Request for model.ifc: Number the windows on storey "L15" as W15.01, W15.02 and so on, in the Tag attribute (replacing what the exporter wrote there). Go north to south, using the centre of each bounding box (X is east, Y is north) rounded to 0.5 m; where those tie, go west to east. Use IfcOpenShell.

First a look at what the model holds.

```python
import ifcopenshell
import ifcopenshell.util.element
import ifcopenshell.util.placement

model = ifcopenshell.open("model.ifc")
print(model.schema)
storey = next(s for s in model.by_type("IfcBuildingStorey") if s.Name == "L15")
windows = [e for e in ifcopenshell.util.element.get_decomposition(storey) if e.is_a("IfcWindow")]
for e in sorted(windows, key=lambda e: e.id()):
    origin = ifcopenshell.util.placement.get_local_placement(e.ObjectPlacement)[:3, 3]
    print(e.id(), e.Tag, e.Name, origin.round(2) + 0.0, sep=" | ")
```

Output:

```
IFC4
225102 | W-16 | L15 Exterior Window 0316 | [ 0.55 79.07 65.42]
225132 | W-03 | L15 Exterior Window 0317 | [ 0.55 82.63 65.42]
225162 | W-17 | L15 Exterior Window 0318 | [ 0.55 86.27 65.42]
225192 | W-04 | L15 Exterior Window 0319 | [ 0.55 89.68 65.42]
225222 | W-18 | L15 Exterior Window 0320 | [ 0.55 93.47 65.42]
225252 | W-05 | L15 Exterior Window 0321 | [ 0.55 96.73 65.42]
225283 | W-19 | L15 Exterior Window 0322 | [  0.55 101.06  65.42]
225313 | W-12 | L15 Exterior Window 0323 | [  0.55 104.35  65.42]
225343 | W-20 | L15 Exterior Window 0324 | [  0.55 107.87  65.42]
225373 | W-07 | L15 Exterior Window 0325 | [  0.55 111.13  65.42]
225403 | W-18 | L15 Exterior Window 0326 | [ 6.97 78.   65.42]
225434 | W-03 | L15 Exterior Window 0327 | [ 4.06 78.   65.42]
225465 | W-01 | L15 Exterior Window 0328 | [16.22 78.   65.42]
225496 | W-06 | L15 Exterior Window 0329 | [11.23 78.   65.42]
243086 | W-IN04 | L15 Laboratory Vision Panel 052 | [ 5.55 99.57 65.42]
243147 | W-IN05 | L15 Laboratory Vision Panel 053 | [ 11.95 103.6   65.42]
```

```python
import ifcopenshell
import ifcopenshell.geom
import ifcopenshell.util.element
import ifcopenshell.util.shape

model = ifcopenshell.open("model.ifc")
settings = ifcopenshell.geom.settings()
settings.set("use-world-coords", True)


def centre(element):
    shape = ifcopenshell.geom.create_shape(settings, element)
    return ifcopenshell.util.shape.get_bbox_centroid(shape.geometry)


storey = next(s for s in model.by_type("IfcBuildingStorey") if s.Name == "L15")
windows = [e for e in ifcopenshell.util.element.get_decomposition(storey) if e.is_a("IfcWindow")]

# Insertion points can sit at a corner or the storey origin, so sort by the geometry (in metres).
centres = {e: centre(e) for e in windows}
windows.sort(key=lambda e: (-round(centres[e][1] / 0.5), centres[e][0]))

for i, e in enumerate(windows, start=1):
    number = f"W15.{i:02d}"
    e.Tag = number
    print(e.id(), number)

model.write("model_rev.ifc")
```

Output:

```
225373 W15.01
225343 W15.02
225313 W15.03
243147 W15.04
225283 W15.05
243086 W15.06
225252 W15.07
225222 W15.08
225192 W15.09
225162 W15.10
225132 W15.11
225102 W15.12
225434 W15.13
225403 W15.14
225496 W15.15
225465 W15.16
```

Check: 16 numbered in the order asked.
